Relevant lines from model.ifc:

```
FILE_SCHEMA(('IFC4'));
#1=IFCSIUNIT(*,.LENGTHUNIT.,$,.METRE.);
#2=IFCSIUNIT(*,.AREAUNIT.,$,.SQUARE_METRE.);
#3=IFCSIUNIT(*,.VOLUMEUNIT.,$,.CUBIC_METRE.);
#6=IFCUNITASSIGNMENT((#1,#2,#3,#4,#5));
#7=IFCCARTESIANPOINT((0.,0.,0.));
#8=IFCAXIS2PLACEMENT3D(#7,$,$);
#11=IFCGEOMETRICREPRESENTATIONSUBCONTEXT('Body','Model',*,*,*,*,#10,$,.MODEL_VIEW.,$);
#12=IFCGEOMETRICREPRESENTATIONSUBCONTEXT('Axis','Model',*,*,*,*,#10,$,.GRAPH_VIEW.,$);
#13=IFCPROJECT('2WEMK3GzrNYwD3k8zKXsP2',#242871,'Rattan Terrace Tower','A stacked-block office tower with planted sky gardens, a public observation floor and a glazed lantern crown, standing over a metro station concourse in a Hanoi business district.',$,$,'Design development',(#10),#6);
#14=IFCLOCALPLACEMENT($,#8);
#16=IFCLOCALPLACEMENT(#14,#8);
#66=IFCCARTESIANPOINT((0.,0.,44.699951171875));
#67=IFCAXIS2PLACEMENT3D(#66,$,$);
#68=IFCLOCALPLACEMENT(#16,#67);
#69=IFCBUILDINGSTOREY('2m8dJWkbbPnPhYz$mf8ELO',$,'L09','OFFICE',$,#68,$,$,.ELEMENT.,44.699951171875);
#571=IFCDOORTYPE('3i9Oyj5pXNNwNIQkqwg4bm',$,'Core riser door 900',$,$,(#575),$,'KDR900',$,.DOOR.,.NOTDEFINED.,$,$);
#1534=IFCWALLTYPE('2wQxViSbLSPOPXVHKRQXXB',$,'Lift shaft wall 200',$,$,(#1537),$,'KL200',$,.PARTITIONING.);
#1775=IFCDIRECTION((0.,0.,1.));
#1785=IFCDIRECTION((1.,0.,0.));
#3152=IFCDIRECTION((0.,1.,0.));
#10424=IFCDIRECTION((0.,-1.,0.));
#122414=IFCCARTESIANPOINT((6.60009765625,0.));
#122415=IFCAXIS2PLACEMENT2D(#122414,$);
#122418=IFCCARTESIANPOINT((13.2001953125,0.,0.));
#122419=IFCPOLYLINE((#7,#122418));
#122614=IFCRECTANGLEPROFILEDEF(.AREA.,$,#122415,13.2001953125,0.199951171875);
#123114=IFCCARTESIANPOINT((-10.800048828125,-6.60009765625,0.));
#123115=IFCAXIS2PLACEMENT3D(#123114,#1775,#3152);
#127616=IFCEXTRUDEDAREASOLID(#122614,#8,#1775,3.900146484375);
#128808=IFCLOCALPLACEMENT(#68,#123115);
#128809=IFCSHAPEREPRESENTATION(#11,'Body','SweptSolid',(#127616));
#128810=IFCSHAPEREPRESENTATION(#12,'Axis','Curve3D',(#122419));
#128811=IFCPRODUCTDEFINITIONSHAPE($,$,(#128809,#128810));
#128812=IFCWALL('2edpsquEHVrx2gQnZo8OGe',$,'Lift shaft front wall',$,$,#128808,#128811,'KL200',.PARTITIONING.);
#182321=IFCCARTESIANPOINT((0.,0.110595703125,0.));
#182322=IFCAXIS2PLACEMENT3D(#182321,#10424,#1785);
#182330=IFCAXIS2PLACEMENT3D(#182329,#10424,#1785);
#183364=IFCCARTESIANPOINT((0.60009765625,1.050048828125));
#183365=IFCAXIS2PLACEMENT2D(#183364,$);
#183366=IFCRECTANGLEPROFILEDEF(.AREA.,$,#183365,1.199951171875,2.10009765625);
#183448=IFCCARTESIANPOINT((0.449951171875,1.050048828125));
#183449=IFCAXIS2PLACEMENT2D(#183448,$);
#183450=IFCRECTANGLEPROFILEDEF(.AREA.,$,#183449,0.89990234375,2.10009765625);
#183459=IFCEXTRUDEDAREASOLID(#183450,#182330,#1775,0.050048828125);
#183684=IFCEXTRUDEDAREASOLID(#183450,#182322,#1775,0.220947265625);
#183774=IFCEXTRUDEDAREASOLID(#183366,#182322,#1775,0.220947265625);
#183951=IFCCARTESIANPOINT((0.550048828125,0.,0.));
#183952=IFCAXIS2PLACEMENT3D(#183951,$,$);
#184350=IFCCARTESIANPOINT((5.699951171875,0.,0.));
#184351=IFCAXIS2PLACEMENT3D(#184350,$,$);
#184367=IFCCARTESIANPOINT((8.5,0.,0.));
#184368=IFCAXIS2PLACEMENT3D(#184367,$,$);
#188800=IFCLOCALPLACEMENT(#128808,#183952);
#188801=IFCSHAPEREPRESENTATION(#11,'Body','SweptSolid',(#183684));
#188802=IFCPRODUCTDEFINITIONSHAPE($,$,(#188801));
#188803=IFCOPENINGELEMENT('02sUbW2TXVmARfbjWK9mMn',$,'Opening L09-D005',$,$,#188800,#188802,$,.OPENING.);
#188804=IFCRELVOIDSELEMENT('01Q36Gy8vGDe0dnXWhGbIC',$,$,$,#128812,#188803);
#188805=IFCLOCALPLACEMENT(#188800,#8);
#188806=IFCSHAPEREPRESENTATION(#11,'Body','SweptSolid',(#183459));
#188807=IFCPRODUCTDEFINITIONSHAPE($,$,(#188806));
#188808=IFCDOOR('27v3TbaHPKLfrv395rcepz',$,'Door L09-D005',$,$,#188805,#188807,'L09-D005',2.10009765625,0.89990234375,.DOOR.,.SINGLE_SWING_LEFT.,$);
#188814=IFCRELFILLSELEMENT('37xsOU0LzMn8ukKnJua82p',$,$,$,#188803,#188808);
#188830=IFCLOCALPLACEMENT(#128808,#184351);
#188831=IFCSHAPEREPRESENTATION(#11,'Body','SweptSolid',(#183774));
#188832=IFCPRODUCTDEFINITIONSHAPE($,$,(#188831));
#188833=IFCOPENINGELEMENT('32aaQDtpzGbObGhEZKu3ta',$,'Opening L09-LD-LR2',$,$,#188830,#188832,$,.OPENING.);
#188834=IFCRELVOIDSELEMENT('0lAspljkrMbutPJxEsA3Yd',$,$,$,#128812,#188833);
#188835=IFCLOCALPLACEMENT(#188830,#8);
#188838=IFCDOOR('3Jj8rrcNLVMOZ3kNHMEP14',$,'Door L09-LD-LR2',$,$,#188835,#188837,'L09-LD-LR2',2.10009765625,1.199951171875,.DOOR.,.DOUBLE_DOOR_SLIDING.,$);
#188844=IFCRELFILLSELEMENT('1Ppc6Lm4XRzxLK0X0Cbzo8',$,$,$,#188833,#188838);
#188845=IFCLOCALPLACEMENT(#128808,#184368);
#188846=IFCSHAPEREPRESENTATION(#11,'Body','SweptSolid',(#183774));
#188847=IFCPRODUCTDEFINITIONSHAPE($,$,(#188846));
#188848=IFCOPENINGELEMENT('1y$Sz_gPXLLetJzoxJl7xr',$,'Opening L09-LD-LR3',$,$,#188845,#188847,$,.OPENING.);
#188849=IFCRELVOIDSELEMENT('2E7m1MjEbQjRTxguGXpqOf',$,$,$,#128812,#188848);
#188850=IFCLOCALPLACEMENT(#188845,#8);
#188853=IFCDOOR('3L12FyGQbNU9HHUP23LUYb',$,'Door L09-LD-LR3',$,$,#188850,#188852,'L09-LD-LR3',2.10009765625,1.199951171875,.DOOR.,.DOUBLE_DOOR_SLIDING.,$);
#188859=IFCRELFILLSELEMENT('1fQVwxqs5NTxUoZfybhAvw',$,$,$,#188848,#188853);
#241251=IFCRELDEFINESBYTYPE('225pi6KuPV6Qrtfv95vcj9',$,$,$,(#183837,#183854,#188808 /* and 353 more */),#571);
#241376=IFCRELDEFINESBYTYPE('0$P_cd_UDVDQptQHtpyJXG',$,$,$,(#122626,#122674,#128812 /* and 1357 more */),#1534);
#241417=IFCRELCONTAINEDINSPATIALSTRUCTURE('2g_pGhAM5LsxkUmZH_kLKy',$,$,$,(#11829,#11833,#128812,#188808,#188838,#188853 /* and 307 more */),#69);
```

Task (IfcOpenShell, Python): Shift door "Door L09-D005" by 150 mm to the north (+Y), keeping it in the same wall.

```python
import ifcopenshell
import ifcopenshell.api.geometry
import ifcopenshell.util.placement

model = ifcopenshell.open("model.ifc")

door = model.by_guid("27v3TbaHPKLfrv395rcepz")
opening = door.FillsVoids[0].RelatingOpeningElement
wall = opening.VoidsElements[0].RelatingBuildingElement

wall_matrix = ifcopenshell.util.placement.get_local_placement(wall.ObjectPlacement)
shift = wall_matrix[:3, 0] * 0.15
before = ifcopenshell.util.placement.get_local_placement(door.ObjectPlacement)[:3, 3].copy()

# The door is placed relative to its opening, so it follows when the opening moves.
matrix = ifcopenshell.util.placement.get_local_placement(opening.ObjectPlacement)
matrix[:3, 3] += shift
ifcopenshell.api.geometry.edit_object_placement(
    model, product=opening, matrix=matrix, is_si=False, should_transform_children=True
)

after = ifcopenshell.util.placement.get_local_placement(door.ObjectPlacement)[:3, 3]
print("door moved by", (after - before).round(3) + 0.0)

model.write("model-out.ifc")
```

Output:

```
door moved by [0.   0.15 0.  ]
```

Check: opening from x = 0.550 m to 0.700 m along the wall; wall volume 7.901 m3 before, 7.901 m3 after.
